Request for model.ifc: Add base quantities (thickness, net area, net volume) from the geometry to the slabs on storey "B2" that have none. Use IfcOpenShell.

First a look at what the model holds.

```python
import ifcopenshell
import ifcopenshell.util.element
import ifcopenshell.util.unit

model = ifcopenshell.open("model.ifc")
print(model.schema)
for unit_type in ("LENGTHUNIT", "AREAUNIT", "VOLUMEUNIT"):
    print(unit_type, ifcopenshell.util.unit.calculate_unit_scale(model, unit_type))
storey = next(s for s in model.by_type("IfcBuildingStorey") if s.Name == "B2")
slabs = [e for e in ifcopenshell.util.element.get_decomposition(storey) if e.is_a("IfcSlab")]
for e in sorted(slabs, key=lambda e: e.id()):
    print(e.id(), e.is_a(), e.Name, list(ifcopenshell.util.element.get_psets(e, qtos_only=True)), sep=" | ")
```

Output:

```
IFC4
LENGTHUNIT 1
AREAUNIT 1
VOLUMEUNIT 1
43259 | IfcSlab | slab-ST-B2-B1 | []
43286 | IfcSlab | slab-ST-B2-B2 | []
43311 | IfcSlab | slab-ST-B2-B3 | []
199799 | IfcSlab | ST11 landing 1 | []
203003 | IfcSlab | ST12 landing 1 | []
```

```python
import ifcopenshell
import ifcopenshell.api.pset
import ifcopenshell.geom
import ifcopenshell.util.element
import ifcopenshell.util.shape
import ifcopenshell.util.unit

model = ifcopenshell.open("model.ifc")
unit_scale = ifcopenshell.util.unit.calculate_unit_scale(model)
area_scale = ifcopenshell.util.unit.calculate_unit_scale(model, "AREAUNIT")
volume_scale = ifcopenshell.util.unit.calculate_unit_scale(model, "VOLUMEUNIT")
settings = ifcopenshell.geom.settings()

storey = next(s for s in model.by_type("IfcBuildingStorey") if s.Name == "B2")
slabs = [e for e in ifcopenshell.util.element.get_decomposition(storey) if e.is_a("IfcSlab")]

for e in sorted(slabs, key=lambda e: e.id()):
    if ifcopenshell.util.element.get_psets(e, qtos_only=True, should_inherit=False):
        continue
    # Geometry comes back in metres, in the element's own axes.
    shape = ifcopenshell.geom.create_shape(settings, e)
    values = {
        "Width": ifcopenshell.util.shape.get_z(shape.geometry) / unit_scale,
        "NetArea": ifcopenshell.util.shape.get_footprint_area(shape.geometry) / area_scale,
        "NetVolume": ifcopenshell.util.shape.get_volume(shape.geometry) / volume_scale,
    }
    qto = ifcopenshell.api.pset.add_qto(model, product=e, name="Qto_SlabBaseQuantities")
    ifcopenshell.api.pset.edit_qto(model, qto=qto, properties=values)
    print(e.id(), {k: round(v, 3) for k, v in values.items()})

model.write("model_rev.ifc")
```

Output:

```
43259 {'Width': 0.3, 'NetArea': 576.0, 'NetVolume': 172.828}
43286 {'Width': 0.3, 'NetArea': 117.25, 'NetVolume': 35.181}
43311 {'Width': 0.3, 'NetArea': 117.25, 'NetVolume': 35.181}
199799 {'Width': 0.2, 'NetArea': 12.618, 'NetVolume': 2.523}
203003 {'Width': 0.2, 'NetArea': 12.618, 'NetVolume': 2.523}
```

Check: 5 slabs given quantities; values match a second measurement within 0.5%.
